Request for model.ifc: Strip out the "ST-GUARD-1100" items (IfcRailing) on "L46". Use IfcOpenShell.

First a look at what the model holds.

```python
import ifcopenshell
import ifcopenshell.util.element

model = ifcopenshell.open("model.ifc")
print(model.schema)
storey = next(s for s in model.by_type("IfcBuildingStorey") if s.Name == "L46")
railings = [e for e in ifcopenshell.util.element.get_decomposition(storey) if e.is_a("IfcRailing")]
seen = {}
for e in railings:
    element_type = ifcopenshell.util.element.get_type(e)
    name = element_type.Name if element_type not in (None, e) else None
    seen[name] = seen.get(name, 0) + 1
for name, count in sorted(seen.items(), key=str):
    print(count, "x", name)
```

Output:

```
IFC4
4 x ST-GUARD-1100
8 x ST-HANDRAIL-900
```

```python
import ifcopenshell
import ifcopenshell.api.root
import ifcopenshell.util.element

model = ifcopenshell.open("model.ifc")

storey = next(s for s in model.by_type("IfcBuildingStorey") if s.Name == "L46")
railings = [e for e in ifcopenshell.util.element.get_decomposition(storey) if e.is_a("IfcRailing")]
targets = [e for e in railings if (t := ifcopenshell.util.element.get_type(e)) not in (None, e) and t.Name == "ST-GUARD-1100"]

for e in targets:
    ifcopenshell.api.root.remove_product(model, product=e)
print(len(targets), "removed")

model.write("model_v2.ifc")
```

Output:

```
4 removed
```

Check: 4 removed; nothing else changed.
